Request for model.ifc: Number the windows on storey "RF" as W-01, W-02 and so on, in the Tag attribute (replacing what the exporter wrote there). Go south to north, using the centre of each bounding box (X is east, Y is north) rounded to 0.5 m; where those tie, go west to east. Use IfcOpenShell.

First a look at what the model holds.

```python
import ifcopenshell
import ifcopenshell.util.element
import ifcopenshell.util.placement

model = ifcopenshell.open("model.ifc")
print(model.schema)
storey = next(s for s in model.by_type("IfcBuildingStorey") if s.Name == "RF")
windows = [e for e in ifcopenshell.util.element.get_decomposition(storey) if e.is_a("IfcWindow")]
for e in sorted(windows, key=lambda e: e.id()):
    origin = ifcopenshell.util.placement.get_local_placement(e.ObjectPlacement)[:3, 3]
    print(e.id(), e.Tag, e.Name, origin.round(2) + 0.0, sep=" | ")
```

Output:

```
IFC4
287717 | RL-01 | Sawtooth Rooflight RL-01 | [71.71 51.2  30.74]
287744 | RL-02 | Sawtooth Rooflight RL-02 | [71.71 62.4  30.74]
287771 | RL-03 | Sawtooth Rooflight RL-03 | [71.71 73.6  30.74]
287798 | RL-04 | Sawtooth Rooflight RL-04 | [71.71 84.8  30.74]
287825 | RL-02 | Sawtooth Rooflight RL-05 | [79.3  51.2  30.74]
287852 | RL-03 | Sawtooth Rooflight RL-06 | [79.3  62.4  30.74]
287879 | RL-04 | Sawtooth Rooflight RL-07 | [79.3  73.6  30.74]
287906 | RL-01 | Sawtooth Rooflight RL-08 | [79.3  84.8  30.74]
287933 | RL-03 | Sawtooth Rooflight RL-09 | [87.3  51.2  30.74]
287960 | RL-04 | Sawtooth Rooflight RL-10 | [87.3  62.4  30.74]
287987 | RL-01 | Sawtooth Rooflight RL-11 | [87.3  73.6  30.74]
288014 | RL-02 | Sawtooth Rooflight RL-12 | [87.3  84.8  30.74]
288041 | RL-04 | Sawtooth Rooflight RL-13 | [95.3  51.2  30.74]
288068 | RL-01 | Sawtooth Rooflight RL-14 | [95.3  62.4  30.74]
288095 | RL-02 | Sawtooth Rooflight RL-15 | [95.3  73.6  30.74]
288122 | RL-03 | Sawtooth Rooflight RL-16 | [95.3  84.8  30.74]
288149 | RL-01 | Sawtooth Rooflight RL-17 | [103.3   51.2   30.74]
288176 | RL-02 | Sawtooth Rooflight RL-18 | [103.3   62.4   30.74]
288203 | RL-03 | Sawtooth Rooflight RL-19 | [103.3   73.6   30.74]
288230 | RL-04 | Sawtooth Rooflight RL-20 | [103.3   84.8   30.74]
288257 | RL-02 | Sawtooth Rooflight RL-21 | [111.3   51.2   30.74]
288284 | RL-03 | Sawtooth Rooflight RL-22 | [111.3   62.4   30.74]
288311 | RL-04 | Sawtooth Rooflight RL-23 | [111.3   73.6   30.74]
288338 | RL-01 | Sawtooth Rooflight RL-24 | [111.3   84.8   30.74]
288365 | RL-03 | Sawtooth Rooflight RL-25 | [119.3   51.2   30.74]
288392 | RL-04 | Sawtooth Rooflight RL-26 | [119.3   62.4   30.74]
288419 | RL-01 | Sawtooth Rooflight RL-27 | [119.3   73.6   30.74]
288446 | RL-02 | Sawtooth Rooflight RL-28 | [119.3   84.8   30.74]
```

```python
import ifcopenshell
import ifcopenshell.geom
import ifcopenshell.util.element
import ifcopenshell.util.shape

model = ifcopenshell.open("model.ifc")
settings = ifcopenshell.geom.settings()
settings.set("use-world-coords", True)


def centre(element):
    shape = ifcopenshell.geom.create_shape(settings, element)
    return ifcopenshell.util.shape.get_bbox_centroid(shape.geometry)


storey = next(s for s in model.by_type("IfcBuildingStorey") if s.Name == "RF")
windows = [e for e in ifcopenshell.util.element.get_decomposition(storey) if e.is_a("IfcWindow")]

# Insertion points can sit at a corner or the storey origin, so sort by the geometry (in metres).
centres = {e: centre(e) for e in windows}
windows.sort(key=lambda e: (round(centres[e][1] / 0.5), centres[e][0]))

for i, e in enumerate(windows, start=1):
    number = f"W-{i:02d}"
    e.Tag = number
    print(e.id(), number)

model.write("model_v2.ifc")
```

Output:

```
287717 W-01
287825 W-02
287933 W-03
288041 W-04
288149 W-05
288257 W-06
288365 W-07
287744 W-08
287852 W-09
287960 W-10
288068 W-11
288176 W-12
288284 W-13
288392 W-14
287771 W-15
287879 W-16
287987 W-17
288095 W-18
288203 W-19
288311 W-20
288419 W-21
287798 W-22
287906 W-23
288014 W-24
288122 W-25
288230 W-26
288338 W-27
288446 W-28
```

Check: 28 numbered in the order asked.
